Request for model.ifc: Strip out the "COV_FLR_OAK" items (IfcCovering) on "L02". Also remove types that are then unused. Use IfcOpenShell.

First a look at what the model holds.

```python
import ifcopenshell
import ifcopenshell.util.element

model = ifcopenshell.open("model.ifc")
print(model.schema)
storey = next(s for s in model.by_type("IfcBuildingStorey") if s.Name == "L02")
coverings = [e for e in ifcopenshell.util.element.get_decomposition(storey) if e.is_a("IfcCovering")]
seen = {}
for e in coverings:
    element_type = ifcopenshell.util.element.get_type(e)
    name = element_type.Name if element_type not in (None, e) else None
    seen[name] = seen.get(name, 0) + 1
for name, count in sorted(seen.items(), key=str):
    print(count, "x", name)
```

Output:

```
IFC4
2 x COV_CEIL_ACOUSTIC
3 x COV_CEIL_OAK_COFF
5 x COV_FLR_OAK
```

```python
import ifcopenshell
import ifcopenshell.api.root
import ifcopenshell.util.element

model = ifcopenshell.open("model.ifc")

storey = next(s for s in model.by_type("IfcBuildingStorey") if s.Name == "L02")
coverings = [e for e in ifcopenshell.util.element.get_decomposition(storey) if e.is_a("IfcCovering")]
targets = [e for e in coverings if (t := ifcopenshell.util.element.get_type(e)) not in (None, e) and t.Name == "COV_FLR_OAK"]
types = {ifcopenshell.util.element.get_type(e) for e in targets} - {None, *targets}

for e in targets:
    ifcopenshell.api.root.remove_product(model, product=e)
print(len(targets), "removed")

unused = [t for t in types if not ifcopenshell.util.element.get_types(t)]
for t in unused:
    ifcopenshell.api.root.remove_product(model, product=t)
print(len(unused), "unused types removed")

model.write("model_edited.ifc")
```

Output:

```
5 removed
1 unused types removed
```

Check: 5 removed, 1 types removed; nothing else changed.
